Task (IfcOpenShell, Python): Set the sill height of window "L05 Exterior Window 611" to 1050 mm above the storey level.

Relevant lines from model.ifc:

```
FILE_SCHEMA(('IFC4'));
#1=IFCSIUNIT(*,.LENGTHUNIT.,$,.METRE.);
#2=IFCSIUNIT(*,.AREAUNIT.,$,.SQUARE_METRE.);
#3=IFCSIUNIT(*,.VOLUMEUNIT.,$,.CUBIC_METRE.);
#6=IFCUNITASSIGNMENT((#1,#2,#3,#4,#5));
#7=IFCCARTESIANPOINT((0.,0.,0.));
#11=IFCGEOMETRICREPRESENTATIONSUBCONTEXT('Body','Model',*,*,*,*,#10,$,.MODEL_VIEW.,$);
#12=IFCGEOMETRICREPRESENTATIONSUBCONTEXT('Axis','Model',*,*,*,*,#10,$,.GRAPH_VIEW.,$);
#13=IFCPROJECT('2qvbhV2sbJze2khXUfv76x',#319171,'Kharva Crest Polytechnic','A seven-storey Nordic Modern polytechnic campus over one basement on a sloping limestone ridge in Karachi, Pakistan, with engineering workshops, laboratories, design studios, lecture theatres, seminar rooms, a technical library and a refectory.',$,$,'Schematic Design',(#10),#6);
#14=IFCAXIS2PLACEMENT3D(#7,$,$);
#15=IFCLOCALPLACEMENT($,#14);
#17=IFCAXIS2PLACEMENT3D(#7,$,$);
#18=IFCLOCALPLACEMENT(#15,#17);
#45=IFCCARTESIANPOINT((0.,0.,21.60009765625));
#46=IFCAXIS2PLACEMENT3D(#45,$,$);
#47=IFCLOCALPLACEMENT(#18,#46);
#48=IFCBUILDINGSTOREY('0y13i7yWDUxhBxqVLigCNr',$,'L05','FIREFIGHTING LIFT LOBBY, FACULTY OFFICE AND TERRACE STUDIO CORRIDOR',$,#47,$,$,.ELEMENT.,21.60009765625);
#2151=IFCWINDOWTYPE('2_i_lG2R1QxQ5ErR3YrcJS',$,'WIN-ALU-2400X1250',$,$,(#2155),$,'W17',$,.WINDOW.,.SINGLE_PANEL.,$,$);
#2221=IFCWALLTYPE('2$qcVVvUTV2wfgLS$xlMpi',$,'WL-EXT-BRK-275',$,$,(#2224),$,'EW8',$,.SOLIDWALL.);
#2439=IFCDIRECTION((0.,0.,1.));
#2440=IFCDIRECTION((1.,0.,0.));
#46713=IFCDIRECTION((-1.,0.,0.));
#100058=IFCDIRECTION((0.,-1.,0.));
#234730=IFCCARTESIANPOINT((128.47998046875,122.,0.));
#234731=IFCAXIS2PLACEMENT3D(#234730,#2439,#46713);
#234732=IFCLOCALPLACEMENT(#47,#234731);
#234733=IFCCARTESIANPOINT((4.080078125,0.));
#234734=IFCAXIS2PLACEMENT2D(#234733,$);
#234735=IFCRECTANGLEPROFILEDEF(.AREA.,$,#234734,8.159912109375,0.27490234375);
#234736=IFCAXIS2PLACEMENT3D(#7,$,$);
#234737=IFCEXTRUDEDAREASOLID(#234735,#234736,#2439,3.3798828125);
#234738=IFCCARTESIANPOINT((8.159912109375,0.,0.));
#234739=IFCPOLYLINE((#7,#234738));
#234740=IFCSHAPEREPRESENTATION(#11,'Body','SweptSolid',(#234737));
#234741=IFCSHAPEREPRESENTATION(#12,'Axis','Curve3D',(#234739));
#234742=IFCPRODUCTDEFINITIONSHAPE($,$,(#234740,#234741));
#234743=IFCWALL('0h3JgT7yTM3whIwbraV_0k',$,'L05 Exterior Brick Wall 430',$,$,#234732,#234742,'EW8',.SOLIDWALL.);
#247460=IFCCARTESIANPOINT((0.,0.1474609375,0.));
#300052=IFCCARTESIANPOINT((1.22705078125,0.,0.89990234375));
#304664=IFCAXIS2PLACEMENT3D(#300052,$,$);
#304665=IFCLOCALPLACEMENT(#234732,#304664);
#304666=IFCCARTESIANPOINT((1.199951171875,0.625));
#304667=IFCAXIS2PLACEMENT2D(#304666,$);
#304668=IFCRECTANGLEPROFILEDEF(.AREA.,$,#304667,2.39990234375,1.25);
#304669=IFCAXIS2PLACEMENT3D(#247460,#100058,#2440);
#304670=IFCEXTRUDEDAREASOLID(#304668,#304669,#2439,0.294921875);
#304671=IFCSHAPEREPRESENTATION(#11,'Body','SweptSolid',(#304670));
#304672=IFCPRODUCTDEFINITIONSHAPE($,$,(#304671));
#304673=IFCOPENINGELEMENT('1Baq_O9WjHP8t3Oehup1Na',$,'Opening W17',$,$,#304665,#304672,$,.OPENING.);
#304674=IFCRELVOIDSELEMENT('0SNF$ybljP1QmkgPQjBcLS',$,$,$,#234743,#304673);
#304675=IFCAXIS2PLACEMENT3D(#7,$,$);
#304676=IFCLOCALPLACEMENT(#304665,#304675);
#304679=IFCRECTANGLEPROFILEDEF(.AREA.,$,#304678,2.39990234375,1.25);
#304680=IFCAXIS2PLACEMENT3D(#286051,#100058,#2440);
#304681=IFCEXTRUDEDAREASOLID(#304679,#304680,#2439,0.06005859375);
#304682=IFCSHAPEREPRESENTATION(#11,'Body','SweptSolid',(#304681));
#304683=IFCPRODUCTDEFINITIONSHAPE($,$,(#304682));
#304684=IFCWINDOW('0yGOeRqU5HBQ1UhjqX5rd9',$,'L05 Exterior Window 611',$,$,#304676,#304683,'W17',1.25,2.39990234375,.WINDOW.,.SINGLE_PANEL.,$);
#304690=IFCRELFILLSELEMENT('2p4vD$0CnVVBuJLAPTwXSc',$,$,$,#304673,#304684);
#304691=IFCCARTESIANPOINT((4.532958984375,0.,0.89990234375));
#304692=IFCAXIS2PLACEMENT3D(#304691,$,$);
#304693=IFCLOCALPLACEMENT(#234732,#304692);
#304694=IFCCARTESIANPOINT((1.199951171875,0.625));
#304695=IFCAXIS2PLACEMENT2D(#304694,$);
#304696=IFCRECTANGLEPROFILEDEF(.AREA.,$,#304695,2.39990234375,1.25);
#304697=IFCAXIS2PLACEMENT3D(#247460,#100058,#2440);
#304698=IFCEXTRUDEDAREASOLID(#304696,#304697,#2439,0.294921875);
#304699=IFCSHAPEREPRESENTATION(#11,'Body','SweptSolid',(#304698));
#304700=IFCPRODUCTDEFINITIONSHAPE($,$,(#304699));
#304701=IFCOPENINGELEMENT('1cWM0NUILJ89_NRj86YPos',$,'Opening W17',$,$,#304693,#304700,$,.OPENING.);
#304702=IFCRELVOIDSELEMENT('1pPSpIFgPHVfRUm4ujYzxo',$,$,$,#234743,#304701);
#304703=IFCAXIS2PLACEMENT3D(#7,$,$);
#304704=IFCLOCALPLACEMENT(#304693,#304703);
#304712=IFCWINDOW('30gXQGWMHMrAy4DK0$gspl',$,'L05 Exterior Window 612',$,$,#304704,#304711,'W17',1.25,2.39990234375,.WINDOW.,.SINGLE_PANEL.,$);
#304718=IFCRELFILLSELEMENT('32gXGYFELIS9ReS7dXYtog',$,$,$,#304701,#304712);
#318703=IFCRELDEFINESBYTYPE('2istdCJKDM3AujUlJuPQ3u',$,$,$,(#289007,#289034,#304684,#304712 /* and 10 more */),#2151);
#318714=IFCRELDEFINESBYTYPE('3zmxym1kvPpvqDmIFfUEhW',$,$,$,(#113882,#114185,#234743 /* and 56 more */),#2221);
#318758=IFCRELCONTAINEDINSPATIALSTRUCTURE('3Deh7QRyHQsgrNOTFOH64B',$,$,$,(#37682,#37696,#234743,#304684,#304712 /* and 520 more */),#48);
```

```python
import numpy as np
import ifcopenshell
import ifcopenshell.api.geometry
import ifcopenshell.geom
import ifcopenshell.util.element
import ifcopenshell.util.placement
import ifcopenshell.util.shape
import ifcopenshell.util.unit

model = ifcopenshell.open("model.ifc")
unit_scale = ifcopenshell.util.unit.calculate_unit_scale(model)

window = model.by_guid("0yGOeRqU5HBQ1UhjqX5rd9")
opening = window.FillsVoids[0].RelatingOpeningElement
storey = ifcopenshell.util.element.get_container(window, ifc_class="IfcBuildingStorey")
level = ifcopenshell.util.placement.get_local_placement(storey.ObjectPlacement)[2, 3]

# The opening's origin need not be at the sill, so measure its lowest point.
shape = ifcopenshell.geom.create_shape(ifcopenshell.geom.settings(), opening)
bottom = ifcopenshell.util.shape.get_shape_bottom_elevation(shape, shape.geometry) / unit_scale
dz = level + 1.05 / unit_scale - bottom

shift = np.array([0.0, 0.0, dz])
# The window is placed relative to its opening, so it follows when the opening moves.
matrix = ifcopenshell.util.placement.get_local_placement(opening.ObjectPlacement)
matrix[:3, 3] += shift
ifcopenshell.api.geometry.edit_object_placement(
    model, product=opening, matrix=matrix, is_si=False, should_transform_children=True
)

print(f"moved by {dz * unit_scale:+.3f} m")

model.write("model-out.ifc")
```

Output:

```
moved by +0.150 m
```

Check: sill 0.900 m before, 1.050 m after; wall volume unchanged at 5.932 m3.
